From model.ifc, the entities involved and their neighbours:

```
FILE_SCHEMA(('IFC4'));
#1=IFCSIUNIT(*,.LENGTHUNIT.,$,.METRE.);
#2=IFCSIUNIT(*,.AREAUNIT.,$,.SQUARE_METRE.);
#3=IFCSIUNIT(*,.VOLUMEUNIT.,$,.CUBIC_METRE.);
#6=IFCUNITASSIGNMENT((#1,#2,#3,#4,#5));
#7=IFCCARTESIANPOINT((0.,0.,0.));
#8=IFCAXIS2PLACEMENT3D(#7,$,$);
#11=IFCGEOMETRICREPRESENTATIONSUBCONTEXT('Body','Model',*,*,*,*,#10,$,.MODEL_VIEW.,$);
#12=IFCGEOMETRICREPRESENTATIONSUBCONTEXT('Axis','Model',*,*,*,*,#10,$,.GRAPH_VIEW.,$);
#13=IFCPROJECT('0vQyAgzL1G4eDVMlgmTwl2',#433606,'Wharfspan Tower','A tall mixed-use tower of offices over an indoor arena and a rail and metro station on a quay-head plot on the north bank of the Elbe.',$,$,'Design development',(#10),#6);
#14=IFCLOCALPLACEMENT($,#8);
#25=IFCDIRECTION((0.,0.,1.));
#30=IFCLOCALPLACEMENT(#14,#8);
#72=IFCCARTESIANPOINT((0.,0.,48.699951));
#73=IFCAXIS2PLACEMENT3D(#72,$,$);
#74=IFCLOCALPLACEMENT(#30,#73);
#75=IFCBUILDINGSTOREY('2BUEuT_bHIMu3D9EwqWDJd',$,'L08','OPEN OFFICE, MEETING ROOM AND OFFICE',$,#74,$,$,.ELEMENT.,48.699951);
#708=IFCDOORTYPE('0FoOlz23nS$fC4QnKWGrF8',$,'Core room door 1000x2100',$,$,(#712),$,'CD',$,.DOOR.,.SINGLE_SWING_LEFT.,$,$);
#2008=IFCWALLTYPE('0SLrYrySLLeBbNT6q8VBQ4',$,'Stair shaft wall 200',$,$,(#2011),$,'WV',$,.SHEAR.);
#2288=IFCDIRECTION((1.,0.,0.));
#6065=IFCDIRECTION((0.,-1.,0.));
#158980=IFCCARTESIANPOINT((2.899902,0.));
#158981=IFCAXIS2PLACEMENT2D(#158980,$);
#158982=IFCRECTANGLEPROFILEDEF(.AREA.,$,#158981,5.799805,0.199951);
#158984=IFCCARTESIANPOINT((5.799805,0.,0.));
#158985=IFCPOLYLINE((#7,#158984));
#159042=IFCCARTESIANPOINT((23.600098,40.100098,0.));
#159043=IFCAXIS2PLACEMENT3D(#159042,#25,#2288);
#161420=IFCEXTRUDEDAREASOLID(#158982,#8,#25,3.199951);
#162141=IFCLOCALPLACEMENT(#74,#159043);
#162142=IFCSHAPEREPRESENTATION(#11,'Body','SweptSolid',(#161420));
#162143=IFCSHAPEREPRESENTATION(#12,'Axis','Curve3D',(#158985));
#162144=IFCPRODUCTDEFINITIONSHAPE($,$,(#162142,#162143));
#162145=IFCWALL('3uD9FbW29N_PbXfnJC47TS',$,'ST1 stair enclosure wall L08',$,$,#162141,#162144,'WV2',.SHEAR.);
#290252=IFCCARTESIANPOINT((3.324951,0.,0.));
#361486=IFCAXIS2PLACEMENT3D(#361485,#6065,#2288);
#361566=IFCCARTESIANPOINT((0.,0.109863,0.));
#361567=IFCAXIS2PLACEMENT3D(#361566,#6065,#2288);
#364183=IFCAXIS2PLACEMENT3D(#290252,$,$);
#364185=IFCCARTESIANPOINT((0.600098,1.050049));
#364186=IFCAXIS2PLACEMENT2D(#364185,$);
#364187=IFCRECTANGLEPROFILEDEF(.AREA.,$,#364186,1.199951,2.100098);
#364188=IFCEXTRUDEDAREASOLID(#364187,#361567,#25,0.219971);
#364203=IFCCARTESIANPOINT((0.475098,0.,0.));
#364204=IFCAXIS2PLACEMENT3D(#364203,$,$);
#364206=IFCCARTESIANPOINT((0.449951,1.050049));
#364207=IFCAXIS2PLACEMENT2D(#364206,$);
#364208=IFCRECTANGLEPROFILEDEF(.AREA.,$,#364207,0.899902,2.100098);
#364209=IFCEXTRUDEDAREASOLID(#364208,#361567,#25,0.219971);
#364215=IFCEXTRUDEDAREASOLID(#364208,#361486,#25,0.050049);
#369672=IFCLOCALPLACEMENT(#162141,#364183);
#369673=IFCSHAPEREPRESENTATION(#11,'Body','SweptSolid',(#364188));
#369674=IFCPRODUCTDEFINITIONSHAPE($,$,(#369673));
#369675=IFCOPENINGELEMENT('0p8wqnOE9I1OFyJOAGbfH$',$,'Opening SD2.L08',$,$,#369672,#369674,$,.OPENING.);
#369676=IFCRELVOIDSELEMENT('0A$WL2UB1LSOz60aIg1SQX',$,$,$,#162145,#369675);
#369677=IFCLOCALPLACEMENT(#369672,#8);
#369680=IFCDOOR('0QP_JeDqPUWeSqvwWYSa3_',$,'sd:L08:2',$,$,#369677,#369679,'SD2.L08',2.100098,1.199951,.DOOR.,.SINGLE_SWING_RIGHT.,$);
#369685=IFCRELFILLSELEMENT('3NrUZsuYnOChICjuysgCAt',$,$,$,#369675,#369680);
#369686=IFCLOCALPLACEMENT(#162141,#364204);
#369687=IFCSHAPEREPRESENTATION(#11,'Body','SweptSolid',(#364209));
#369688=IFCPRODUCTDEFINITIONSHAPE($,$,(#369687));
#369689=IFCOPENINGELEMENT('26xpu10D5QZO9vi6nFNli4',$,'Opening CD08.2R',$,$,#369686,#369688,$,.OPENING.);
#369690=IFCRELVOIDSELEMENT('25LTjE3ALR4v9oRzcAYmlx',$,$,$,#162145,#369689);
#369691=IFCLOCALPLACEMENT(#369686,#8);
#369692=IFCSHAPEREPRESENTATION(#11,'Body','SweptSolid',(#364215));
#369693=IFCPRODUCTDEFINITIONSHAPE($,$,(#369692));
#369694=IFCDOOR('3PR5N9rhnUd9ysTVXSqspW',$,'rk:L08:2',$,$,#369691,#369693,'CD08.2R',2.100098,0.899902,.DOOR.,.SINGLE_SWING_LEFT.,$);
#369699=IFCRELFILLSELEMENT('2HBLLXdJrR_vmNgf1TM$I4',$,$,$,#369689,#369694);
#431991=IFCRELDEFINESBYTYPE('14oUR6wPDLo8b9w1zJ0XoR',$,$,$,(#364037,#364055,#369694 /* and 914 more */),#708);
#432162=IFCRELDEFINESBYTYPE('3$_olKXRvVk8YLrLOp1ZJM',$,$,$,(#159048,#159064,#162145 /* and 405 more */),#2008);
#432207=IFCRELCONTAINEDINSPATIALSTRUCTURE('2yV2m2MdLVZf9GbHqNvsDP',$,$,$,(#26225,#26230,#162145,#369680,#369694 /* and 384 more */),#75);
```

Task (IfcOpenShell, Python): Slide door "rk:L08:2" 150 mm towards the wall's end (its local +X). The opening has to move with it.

```python
import ifcopenshell
import ifcopenshell.api.geometry
import ifcopenshell.util.placement

model = ifcopenshell.open("model.ifc")

door = model.by_guid("3PR5N9rhnUd9ysTVXSqspW")
opening = door.FillsVoids[0].RelatingOpeningElement
wall = opening.VoidsElements[0].RelatingBuildingElement

wall_matrix = ifcopenshell.util.placement.get_local_placement(wall.ObjectPlacement)
shift = wall_matrix[:3, 0] * 0.15
before = ifcopenshell.util.placement.get_local_placement(door.ObjectPlacement)[:3, 3].copy()

# The door is placed relative to its opening, so it follows when the opening moves.
matrix = ifcopenshell.util.placement.get_local_placement(opening.ObjectPlacement)
matrix[:3, 3] += shift
ifcopenshell.api.geometry.edit_object_placement(
    model, product=opening, matrix=matrix, is_si=False, should_transform_children=True
)

after = ifcopenshell.util.placement.get_local_placement(door.ObjectPlacement)[:3, 3]
print("door moved by", (after - before).round(3) + 0.0)

model.write("model_v2.ifc")
```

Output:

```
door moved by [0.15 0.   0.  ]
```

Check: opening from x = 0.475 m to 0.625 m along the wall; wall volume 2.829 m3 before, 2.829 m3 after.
